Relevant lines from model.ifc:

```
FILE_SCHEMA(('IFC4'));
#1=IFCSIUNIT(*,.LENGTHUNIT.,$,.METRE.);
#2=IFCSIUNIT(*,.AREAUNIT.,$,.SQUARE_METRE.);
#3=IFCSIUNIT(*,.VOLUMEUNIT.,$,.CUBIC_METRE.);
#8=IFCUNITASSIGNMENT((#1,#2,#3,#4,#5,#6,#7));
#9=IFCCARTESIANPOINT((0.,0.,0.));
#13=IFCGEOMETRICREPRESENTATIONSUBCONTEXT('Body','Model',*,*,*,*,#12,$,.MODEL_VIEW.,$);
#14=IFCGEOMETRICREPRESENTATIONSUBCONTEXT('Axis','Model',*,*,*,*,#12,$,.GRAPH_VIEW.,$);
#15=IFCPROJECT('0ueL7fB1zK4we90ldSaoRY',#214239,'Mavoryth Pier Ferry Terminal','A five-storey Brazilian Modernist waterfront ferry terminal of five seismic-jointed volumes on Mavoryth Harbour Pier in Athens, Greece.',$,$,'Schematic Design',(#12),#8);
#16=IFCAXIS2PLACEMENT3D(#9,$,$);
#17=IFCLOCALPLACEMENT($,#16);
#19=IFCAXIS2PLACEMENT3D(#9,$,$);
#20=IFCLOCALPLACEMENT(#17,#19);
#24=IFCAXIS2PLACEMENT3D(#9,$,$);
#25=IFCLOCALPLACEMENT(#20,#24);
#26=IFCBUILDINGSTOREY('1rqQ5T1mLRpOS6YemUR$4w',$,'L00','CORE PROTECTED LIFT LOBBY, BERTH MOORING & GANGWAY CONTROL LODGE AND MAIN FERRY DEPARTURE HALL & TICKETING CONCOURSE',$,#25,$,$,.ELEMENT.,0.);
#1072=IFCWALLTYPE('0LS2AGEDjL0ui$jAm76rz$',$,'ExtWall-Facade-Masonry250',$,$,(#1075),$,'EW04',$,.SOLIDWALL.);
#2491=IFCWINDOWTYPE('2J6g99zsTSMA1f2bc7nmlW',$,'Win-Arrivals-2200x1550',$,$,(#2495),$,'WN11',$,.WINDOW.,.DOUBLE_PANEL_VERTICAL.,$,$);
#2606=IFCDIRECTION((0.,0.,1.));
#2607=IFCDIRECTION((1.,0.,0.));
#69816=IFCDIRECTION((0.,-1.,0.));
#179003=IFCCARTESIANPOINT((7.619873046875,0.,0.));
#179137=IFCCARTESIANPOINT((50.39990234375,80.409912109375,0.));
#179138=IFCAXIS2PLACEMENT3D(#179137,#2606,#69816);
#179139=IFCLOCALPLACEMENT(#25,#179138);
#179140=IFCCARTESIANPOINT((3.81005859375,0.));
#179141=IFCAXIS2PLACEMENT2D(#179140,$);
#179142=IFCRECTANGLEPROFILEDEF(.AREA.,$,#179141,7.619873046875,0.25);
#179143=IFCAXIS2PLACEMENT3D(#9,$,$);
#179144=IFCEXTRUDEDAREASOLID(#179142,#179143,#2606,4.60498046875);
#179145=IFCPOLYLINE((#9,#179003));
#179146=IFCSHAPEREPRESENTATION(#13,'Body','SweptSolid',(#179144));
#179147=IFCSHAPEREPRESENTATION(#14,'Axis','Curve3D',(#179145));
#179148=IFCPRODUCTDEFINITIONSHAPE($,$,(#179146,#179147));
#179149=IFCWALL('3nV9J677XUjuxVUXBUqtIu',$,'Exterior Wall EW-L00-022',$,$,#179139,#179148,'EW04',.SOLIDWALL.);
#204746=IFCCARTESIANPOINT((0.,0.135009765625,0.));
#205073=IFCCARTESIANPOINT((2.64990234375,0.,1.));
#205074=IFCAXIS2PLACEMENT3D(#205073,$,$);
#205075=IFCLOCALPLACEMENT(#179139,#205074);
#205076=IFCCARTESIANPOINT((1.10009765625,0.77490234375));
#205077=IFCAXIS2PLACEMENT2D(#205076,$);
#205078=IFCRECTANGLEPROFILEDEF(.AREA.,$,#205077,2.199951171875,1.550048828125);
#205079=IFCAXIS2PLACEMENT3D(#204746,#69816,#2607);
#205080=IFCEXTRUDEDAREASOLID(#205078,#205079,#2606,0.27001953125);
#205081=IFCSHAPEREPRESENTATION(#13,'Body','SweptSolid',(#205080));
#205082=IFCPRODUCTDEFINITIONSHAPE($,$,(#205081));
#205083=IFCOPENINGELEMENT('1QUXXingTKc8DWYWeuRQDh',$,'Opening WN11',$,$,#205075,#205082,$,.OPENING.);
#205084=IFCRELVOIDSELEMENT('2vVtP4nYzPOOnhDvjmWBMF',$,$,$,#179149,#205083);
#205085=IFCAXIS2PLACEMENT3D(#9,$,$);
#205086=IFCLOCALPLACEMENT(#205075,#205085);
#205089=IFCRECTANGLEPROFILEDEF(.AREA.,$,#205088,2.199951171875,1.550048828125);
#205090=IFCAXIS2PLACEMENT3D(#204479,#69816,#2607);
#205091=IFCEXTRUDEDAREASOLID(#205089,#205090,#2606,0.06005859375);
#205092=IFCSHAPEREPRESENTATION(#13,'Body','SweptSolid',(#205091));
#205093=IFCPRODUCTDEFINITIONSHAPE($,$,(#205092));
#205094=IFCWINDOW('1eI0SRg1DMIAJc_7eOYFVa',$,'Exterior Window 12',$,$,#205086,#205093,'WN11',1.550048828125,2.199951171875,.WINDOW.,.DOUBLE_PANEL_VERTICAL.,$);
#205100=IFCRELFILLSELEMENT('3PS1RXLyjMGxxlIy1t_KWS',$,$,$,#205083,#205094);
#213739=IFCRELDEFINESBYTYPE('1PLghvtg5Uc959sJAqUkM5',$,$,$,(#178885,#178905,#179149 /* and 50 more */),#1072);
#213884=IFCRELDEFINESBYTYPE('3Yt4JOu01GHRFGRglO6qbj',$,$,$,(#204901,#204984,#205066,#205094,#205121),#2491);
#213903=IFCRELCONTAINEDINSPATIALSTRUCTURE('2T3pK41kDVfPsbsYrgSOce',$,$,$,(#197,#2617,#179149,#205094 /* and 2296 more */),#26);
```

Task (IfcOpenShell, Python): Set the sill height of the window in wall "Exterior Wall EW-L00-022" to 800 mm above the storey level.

```python
import numpy as np
import ifcopenshell
import ifcopenshell.api.geometry
import ifcopenshell.geom
import ifcopenshell.util.element
import ifcopenshell.util.placement
import ifcopenshell.util.shape
import ifcopenshell.util.unit

model = ifcopenshell.open("model.ifc")
unit_scale = ifcopenshell.util.unit.calculate_unit_scale(model)

window = model.by_guid("1eI0SRg1DMIAJc_7eOYFVa")
opening = window.FillsVoids[0].RelatingOpeningElement
storey = ifcopenshell.util.element.get_container(window, ifc_class="IfcBuildingStorey")
level = ifcopenshell.util.placement.get_local_placement(storey.ObjectPlacement)[2, 3]

# The opening's origin need not be at the sill, so measure its lowest point.
shape = ifcopenshell.geom.create_shape(ifcopenshell.geom.settings(), opening)
bottom = ifcopenshell.util.shape.get_shape_bottom_elevation(shape, shape.geometry) / unit_scale
dz = level + 0.8 - bottom

shift = np.array([0.0, 0.0, dz])
# The window is placed relative to its opening, so it follows when the opening moves.
matrix = ifcopenshell.util.placement.get_local_placement(opening.ObjectPlacement)
matrix[:3, 3] += shift
ifcopenshell.api.geometry.edit_object_placement(
    model, product=opening, matrix=matrix, is_si=False, should_transform_children=True
)

print(f"moved by {dz * unit_scale:+.3f} m")

model.write("model_v2.ifc")
```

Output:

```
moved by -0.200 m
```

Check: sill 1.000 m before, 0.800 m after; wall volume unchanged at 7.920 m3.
